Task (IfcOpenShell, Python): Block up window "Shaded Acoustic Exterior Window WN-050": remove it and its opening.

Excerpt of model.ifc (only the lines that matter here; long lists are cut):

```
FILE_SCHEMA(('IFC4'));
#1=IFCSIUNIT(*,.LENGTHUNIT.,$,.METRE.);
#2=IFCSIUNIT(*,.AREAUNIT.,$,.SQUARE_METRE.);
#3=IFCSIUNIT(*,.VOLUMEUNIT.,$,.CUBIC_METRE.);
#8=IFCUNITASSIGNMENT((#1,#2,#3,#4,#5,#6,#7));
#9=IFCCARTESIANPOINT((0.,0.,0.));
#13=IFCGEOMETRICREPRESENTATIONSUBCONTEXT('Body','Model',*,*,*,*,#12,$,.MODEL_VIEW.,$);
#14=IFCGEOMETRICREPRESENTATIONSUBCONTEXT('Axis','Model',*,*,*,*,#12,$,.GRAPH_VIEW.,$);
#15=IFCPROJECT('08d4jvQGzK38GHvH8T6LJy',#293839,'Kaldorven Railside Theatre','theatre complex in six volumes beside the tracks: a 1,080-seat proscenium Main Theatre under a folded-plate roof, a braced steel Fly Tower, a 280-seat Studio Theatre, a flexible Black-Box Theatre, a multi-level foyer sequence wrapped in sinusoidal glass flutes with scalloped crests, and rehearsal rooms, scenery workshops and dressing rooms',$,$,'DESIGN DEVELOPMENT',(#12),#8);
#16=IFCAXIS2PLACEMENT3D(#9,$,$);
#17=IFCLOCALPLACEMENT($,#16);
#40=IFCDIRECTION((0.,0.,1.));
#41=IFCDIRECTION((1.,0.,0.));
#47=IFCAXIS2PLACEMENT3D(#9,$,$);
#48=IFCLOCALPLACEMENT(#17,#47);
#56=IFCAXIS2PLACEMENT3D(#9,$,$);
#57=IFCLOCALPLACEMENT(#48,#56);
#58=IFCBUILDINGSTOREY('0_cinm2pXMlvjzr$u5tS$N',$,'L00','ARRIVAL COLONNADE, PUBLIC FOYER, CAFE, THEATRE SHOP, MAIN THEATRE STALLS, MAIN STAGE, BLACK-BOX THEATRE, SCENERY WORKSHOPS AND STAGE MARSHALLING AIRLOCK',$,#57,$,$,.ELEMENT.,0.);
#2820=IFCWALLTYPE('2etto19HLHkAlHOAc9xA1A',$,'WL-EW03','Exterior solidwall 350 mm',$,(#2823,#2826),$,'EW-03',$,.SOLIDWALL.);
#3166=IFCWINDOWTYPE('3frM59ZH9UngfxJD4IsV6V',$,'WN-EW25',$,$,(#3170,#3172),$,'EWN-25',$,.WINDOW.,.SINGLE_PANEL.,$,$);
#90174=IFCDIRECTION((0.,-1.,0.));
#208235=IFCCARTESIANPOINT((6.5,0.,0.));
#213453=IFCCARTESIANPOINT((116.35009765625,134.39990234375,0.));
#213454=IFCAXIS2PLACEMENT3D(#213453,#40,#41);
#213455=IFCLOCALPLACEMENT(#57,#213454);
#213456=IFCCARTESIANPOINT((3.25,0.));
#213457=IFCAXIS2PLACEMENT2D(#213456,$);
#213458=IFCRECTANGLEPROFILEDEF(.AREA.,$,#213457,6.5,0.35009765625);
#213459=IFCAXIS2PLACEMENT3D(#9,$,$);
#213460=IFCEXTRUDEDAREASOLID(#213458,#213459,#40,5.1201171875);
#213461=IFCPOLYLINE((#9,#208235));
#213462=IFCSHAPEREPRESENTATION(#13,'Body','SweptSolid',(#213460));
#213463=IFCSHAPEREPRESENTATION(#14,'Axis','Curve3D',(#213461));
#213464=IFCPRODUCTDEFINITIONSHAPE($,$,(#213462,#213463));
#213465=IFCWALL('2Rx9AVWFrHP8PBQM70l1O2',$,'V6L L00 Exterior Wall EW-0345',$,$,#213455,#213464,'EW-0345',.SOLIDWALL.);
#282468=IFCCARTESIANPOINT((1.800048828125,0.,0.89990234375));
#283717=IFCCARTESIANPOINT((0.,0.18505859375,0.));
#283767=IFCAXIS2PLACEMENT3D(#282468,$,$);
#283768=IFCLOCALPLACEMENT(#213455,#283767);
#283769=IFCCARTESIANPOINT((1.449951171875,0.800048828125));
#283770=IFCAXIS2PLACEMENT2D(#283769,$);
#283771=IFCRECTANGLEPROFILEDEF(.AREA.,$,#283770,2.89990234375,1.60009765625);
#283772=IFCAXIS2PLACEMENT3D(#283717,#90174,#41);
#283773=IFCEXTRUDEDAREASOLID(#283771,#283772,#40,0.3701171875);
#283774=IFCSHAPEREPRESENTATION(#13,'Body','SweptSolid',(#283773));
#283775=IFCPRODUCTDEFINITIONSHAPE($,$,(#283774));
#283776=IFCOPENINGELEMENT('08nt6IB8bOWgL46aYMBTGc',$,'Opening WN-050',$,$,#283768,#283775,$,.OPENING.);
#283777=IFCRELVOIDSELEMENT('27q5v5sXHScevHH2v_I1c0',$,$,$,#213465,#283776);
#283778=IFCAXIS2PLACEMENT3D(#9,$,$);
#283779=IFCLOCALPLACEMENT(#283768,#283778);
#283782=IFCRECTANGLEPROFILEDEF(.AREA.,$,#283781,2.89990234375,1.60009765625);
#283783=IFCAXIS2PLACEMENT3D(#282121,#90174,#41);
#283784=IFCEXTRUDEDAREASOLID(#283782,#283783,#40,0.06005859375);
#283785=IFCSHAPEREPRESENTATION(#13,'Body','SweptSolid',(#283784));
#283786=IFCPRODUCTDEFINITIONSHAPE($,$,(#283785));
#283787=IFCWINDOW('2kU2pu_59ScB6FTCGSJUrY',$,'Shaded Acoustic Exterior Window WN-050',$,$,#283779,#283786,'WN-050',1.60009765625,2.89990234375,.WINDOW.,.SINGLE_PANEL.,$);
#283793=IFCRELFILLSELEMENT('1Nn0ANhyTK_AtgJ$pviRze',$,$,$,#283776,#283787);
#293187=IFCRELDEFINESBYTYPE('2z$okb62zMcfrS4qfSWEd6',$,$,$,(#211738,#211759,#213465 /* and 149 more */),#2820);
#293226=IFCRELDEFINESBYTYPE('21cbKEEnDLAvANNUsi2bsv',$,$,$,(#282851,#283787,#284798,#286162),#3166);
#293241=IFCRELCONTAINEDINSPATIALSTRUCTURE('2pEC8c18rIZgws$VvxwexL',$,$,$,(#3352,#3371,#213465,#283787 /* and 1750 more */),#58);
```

```python
import ifcopenshell
import ifcopenshell.api.feature
import ifcopenshell.api.root
import ifcopenshell.geom
import ifcopenshell.util.shape

model = ifcopenshell.open("model.ifc")
settings = ifcopenshell.geom.settings()


def volume(element):
    """Net volume in cubic metres, openings subtracted."""
    shape = ifcopenshell.geom.create_shape(settings, element)
    return ifcopenshell.util.shape.get_volume(shape.geometry)


window = model.by_id(283787)
opening = window.FillsVoids[0].RelatingOpeningElement
wall = opening.VoidsElements[0].RelatingBuildingElement
before = volume(wall)

ifcopenshell.api.root.remove_product(model, product=window)
ifcopenshell.api.feature.remove_feature(model, feature=opening)

after = volume(wall)

print(f"wall volume {before:.3f} -> {after:.3f} m3")

model.write("model_rev.ifc")
```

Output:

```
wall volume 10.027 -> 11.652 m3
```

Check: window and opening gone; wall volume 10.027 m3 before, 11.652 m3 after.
